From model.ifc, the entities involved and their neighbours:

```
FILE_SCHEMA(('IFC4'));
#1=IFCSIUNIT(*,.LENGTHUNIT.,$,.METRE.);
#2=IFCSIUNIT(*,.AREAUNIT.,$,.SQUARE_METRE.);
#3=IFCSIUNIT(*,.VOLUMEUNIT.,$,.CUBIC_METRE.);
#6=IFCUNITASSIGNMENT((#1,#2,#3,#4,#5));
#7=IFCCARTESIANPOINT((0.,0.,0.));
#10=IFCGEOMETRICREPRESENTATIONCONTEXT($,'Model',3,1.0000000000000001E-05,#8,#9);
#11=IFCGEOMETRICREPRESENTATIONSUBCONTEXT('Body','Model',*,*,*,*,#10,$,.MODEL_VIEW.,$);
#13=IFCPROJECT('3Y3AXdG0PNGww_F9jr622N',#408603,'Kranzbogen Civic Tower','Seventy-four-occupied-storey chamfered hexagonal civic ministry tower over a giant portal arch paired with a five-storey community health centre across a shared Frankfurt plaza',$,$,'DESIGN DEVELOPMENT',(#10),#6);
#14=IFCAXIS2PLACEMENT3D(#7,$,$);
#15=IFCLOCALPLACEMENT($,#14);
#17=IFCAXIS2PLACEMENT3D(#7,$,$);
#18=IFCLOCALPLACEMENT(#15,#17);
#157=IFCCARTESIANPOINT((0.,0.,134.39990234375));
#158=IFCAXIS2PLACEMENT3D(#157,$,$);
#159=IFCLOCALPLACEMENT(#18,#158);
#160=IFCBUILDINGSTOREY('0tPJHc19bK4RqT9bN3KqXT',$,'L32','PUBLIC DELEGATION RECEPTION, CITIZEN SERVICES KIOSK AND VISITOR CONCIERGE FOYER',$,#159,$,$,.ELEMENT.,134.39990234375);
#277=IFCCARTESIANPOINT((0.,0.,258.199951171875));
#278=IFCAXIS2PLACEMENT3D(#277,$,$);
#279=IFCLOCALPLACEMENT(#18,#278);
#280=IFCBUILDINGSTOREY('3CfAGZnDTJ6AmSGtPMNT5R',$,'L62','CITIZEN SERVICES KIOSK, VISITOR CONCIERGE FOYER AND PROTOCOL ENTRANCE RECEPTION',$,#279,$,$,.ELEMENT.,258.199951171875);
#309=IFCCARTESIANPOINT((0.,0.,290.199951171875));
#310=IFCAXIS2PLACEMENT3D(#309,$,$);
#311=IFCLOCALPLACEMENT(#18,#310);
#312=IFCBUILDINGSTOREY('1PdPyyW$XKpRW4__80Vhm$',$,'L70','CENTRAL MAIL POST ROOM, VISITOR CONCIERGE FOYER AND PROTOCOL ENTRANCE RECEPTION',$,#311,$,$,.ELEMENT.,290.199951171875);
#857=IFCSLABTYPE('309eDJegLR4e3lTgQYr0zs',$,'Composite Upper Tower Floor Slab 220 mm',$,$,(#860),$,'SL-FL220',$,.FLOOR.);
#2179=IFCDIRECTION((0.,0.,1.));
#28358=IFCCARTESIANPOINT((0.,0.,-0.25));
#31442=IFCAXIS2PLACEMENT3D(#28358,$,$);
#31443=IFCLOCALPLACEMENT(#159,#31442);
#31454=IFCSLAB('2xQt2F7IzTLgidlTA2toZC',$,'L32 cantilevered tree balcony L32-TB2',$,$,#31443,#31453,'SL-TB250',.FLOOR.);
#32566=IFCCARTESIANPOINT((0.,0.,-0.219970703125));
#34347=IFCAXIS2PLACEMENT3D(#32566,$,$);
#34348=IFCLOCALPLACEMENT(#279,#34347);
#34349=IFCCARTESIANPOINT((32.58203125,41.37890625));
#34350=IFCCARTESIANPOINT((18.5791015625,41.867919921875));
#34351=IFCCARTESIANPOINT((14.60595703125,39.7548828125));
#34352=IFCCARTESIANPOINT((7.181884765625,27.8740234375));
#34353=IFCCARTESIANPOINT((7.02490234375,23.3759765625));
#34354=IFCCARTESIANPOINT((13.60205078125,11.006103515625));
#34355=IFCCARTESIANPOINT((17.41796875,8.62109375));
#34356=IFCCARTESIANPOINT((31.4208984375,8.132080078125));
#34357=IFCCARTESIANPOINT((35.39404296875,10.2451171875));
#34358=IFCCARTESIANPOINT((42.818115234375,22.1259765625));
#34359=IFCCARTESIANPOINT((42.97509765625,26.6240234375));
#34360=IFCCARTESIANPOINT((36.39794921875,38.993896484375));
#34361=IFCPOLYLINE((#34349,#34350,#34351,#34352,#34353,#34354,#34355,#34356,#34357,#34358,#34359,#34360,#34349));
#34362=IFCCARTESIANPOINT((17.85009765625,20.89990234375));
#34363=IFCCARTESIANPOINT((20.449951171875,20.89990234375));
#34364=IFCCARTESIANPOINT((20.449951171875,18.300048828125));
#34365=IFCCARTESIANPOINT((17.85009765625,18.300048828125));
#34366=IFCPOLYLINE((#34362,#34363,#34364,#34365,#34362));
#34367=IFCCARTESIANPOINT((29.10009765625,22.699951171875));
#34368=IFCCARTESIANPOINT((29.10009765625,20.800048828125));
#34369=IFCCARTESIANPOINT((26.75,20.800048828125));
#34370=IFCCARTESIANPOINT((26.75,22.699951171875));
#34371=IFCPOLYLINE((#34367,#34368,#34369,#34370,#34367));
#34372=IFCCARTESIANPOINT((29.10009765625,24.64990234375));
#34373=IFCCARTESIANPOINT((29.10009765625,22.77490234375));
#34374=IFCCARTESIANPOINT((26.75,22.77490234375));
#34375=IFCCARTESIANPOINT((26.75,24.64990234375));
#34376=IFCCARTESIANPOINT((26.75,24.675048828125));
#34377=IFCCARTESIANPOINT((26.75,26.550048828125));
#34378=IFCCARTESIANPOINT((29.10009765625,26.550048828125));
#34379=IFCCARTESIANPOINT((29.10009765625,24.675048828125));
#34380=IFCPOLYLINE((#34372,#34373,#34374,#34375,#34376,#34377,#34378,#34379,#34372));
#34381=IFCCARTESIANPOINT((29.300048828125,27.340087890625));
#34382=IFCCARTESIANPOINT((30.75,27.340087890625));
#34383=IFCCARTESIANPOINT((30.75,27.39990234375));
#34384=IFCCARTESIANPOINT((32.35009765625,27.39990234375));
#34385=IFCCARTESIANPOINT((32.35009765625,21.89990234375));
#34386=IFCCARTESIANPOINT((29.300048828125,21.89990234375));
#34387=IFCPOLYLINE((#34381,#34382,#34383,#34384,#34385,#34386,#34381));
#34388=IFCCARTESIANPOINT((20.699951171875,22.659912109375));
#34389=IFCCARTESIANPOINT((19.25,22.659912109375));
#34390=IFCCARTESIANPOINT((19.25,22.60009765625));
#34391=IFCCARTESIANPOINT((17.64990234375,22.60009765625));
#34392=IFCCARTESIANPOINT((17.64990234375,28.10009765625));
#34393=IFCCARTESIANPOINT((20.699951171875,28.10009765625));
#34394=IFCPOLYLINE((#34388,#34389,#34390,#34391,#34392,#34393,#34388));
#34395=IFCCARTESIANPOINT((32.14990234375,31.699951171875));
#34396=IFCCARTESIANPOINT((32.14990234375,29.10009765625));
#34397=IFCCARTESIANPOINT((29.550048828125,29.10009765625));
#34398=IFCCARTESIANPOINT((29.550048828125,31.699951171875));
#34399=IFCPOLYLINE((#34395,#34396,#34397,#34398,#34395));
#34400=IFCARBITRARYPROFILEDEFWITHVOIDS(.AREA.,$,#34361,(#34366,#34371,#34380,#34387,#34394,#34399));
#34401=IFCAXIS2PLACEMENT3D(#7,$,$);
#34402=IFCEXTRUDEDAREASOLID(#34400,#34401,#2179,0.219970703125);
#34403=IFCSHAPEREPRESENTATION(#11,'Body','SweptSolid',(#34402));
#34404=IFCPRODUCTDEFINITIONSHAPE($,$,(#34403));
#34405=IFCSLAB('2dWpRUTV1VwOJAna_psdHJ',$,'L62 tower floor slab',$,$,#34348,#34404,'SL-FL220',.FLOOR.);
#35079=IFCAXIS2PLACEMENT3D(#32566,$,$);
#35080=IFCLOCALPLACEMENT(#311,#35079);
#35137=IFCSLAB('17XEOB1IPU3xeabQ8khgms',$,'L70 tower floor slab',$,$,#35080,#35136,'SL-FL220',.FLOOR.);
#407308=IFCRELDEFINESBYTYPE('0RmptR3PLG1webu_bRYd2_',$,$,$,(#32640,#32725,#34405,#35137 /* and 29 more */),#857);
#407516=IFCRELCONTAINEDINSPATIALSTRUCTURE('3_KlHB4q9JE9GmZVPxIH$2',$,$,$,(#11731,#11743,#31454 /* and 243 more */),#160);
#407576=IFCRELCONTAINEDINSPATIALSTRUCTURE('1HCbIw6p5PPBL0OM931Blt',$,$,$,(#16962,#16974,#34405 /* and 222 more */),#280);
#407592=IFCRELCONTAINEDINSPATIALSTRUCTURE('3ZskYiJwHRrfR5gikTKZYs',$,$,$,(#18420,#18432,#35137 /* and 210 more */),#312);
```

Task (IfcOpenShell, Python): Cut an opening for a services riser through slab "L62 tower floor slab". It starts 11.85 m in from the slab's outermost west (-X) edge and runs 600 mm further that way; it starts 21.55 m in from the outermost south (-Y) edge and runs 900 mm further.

```python
import numpy as np
import ifcopenshell
import ifcopenshell.api.feature
import ifcopenshell.api.geometry
import ifcopenshell.api.root
import ifcopenshell.geom
import ifcopenshell.util.placement
import ifcopenshell.util.representation
import ifcopenshell.util.shape
import ifcopenshell.util.unit

model = ifcopenshell.open("model.ifc")
unit_scale = ifcopenshell.util.unit.calculate_unit_scale(model)
settings = ifcopenshell.geom.settings()


def volume(element):
    """Net volume in cubic metres, openings subtracted."""
    shape = ifcopenshell.geom.create_shape(settings, element)
    return ifcopenshell.util.shape.get_volume(shape.geometry)


slab = model.by_guid("2dWpRUTV1VwOJAna_psdHJ")
before = volume(slab)

# Extent in the slab's own axes, in metres. The edges named are its -X and -Y sides.
slab_shape = ifcopenshell.geom.create_shape(settings, slab)
vertices = ifcopenshell.util.shape.get_vertices(slab_shape.geometry)
x_min, y_min, bottom = vertices.min(axis=0)
top = vertices[:, 2].max()

opening = ifcopenshell.api.root.create_entity(model, ifc_class="IfcOpeningElement", name="Services riser opening", predefined_type="OPENING")
context = ifcopenshell.util.representation.get_context(model, "Model", "Body", "MODEL_VIEW")
width, depth = 0.6, 0.9
outline = [(0.0, 0.0), (width, 0.0), (width, depth), (0.0, depth), (0.0, 0.0)]
# Overshoot both faces by 50 mm so the cut is clean.
shape = ifcopenshell.api.geometry.add_slab_representation(
    model, context=context, depth=top - bottom + 0.1, polyline=outline
)
ifcopenshell.api.geometry.assign_representation(model, product=opening, representation=shape)

matrix = ifcopenshell.util.placement.get_local_placement(slab.ObjectPlacement)
matrix[:, 3] = matrix @ np.append(np.array([x_min + 11.85, y_min + 21.55, bottom - 0.05]) / unit_scale, 1.0)
ifcopenshell.api.geometry.edit_object_placement(model, product=opening, matrix=matrix, is_si=False)
ifcopenshell.api.feature.add_feature(model, feature=opening, element=slab)

after = volume(slab)

print(f"slab volume {before:.3f} -> {after:.3f} m3")

model.write("model_updated.ifc")
```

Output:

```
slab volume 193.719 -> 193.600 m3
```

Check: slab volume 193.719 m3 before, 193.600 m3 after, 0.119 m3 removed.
